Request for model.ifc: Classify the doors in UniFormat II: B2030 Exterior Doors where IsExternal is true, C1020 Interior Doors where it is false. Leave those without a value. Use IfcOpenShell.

First a look at what the model holds.

```python
import ifcopenshell
import ifcopenshell.util.element

model = ifcopenshell.open("model.ifc")
print(model.schema)
print("classifications:", [c.Name for c in model.by_type("IfcClassification")])
values = [ifcopenshell.util.element.get_pset(e, "Pset_DoorCommon", "IsExternal") for e in model.by_type("IfcDoor")]
for value in (True, False, None):
    print("IsExternal", value, values.count(value))
```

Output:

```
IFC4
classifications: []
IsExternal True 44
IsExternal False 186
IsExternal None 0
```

```python
import ifcopenshell
import ifcopenshell.api.classification
import ifcopenshell.util.element

model = ifcopenshell.open("model.ifc")

system = ifcopenshell.api.classification.add_classification(model, classification="UniFormat II")

doors = model.by_type("IfcDoor")
external = {e: ifcopenshell.util.element.get_pset(e, "Pset_DoorCommon", "IsExternal") for e in doors}
for flag, code, name in ((True, "B2030", "Exterior Doors"), (False, "C1020", "Interior Doors")):
    products = [e for e in doors if external[e] is flag]
    ifcopenshell.api.classification.add_reference(
        model, products=products, classification=system, identification=code, name=name
    )
    print(code, len(products))

model.write("model_edited.ifc")
```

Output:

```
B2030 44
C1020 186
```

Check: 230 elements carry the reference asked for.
